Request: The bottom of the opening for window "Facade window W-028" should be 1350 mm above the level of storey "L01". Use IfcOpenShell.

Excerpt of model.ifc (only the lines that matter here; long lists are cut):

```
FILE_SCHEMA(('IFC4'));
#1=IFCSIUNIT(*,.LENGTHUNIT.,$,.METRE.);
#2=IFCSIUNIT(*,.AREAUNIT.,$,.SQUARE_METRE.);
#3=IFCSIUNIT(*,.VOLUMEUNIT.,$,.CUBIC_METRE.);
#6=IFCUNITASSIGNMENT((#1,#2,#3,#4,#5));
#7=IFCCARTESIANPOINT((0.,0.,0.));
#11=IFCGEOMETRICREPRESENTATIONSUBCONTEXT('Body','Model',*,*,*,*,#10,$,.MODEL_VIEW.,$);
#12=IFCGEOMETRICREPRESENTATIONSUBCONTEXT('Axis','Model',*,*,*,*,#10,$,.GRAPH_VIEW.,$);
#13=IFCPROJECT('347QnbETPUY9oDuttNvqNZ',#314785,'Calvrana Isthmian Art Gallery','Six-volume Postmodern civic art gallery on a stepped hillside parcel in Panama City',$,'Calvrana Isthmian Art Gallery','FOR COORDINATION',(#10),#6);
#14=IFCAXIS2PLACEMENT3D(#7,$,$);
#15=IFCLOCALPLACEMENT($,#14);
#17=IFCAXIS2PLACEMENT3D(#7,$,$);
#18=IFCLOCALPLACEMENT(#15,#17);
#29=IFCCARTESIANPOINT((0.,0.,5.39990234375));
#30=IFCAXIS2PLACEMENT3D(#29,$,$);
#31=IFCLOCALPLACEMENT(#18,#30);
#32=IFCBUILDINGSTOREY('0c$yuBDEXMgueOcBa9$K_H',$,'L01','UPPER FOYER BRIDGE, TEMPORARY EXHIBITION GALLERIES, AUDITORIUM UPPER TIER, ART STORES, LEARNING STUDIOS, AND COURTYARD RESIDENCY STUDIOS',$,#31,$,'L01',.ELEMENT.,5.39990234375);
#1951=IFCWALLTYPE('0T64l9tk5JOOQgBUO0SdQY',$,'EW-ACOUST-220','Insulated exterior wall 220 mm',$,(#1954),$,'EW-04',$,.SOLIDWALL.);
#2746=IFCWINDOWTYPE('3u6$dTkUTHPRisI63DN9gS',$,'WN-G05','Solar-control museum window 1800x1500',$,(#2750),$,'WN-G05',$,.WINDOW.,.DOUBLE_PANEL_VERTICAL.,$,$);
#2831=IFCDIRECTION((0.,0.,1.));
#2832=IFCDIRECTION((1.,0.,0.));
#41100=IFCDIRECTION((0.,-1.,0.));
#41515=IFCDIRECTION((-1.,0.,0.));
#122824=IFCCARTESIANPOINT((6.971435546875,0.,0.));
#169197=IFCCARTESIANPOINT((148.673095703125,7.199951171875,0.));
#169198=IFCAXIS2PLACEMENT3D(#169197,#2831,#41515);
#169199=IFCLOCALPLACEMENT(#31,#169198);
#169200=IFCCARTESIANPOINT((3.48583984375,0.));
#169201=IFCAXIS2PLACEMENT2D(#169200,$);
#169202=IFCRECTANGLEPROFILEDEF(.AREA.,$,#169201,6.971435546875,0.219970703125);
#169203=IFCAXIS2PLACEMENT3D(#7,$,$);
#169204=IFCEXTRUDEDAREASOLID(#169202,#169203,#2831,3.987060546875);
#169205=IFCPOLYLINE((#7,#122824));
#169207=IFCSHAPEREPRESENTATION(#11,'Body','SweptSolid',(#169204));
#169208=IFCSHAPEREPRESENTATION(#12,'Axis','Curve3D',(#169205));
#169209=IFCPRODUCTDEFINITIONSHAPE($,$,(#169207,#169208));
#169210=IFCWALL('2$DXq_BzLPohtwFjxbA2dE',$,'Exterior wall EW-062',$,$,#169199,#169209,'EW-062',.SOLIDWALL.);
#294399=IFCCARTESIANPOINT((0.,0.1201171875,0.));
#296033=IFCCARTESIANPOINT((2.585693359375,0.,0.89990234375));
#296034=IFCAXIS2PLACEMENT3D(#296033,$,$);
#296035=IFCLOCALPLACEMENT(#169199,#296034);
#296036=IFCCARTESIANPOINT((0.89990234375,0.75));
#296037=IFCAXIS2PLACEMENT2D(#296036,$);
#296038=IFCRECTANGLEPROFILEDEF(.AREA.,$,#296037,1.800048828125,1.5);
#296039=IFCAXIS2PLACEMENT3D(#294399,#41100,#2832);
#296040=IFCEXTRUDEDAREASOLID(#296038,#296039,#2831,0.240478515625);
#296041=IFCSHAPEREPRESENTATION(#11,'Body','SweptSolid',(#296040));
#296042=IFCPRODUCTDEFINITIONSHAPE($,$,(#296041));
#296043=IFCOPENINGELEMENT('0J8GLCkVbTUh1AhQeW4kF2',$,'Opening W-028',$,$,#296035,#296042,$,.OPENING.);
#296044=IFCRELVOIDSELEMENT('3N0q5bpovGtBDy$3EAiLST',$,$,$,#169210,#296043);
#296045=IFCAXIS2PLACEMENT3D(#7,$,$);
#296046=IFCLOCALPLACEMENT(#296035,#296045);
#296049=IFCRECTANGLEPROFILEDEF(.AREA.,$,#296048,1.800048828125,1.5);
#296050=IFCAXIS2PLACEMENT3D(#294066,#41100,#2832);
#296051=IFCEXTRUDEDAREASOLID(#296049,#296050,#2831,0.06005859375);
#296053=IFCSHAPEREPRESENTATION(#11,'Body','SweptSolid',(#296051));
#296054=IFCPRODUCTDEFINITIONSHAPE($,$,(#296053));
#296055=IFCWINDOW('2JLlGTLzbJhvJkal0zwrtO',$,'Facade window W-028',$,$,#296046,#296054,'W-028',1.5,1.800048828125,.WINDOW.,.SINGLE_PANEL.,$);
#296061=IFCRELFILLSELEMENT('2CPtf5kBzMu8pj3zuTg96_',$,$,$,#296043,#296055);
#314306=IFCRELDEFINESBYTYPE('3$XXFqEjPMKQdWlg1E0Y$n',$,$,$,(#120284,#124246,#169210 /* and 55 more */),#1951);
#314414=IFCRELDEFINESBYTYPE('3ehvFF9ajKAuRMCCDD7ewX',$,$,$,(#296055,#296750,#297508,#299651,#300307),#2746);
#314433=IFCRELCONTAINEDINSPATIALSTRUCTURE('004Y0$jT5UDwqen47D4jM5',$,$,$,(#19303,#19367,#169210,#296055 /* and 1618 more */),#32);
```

```python
import numpy as np
import ifcopenshell
import ifcopenshell.api.geometry
import ifcopenshell.geom
import ifcopenshell.util.element
import ifcopenshell.util.placement
import ifcopenshell.util.shape
import ifcopenshell.util.unit

model = ifcopenshell.open("model.ifc")
unit_scale = ifcopenshell.util.unit.calculate_unit_scale(model)

window = model.by_id(296055)
opening = window.FillsVoids[0].RelatingOpeningElement
storey = ifcopenshell.util.element.get_container(window, ifc_class="IfcBuildingStorey")
level = ifcopenshell.util.placement.get_local_placement(storey.ObjectPlacement)[2, 3]

# The opening's origin need not be at the sill, so measure its lowest point.
shape = ifcopenshell.geom.create_shape(ifcopenshell.geom.settings(), opening)
bottom = ifcopenshell.util.shape.get_shape_bottom_elevation(shape, shape.geometry) / unit_scale
dz = level + 1.35 / unit_scale - bottom

shift = np.array([0.0, 0.0, dz])
# The window is placed relative to its opening, so it follows when the opening moves.
matrix = ifcopenshell.util.placement.get_local_placement(opening.ObjectPlacement)
matrix[:3, 3] += shift
ifcopenshell.api.geometry.edit_object_placement(
    model, product=opening, matrix=matrix, is_si=False, should_transform_children=True
)

print(f"moved by {dz * unit_scale:+.3f} m")

model.write("model_updated.ifc")
```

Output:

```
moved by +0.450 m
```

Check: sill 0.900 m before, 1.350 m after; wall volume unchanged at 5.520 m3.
